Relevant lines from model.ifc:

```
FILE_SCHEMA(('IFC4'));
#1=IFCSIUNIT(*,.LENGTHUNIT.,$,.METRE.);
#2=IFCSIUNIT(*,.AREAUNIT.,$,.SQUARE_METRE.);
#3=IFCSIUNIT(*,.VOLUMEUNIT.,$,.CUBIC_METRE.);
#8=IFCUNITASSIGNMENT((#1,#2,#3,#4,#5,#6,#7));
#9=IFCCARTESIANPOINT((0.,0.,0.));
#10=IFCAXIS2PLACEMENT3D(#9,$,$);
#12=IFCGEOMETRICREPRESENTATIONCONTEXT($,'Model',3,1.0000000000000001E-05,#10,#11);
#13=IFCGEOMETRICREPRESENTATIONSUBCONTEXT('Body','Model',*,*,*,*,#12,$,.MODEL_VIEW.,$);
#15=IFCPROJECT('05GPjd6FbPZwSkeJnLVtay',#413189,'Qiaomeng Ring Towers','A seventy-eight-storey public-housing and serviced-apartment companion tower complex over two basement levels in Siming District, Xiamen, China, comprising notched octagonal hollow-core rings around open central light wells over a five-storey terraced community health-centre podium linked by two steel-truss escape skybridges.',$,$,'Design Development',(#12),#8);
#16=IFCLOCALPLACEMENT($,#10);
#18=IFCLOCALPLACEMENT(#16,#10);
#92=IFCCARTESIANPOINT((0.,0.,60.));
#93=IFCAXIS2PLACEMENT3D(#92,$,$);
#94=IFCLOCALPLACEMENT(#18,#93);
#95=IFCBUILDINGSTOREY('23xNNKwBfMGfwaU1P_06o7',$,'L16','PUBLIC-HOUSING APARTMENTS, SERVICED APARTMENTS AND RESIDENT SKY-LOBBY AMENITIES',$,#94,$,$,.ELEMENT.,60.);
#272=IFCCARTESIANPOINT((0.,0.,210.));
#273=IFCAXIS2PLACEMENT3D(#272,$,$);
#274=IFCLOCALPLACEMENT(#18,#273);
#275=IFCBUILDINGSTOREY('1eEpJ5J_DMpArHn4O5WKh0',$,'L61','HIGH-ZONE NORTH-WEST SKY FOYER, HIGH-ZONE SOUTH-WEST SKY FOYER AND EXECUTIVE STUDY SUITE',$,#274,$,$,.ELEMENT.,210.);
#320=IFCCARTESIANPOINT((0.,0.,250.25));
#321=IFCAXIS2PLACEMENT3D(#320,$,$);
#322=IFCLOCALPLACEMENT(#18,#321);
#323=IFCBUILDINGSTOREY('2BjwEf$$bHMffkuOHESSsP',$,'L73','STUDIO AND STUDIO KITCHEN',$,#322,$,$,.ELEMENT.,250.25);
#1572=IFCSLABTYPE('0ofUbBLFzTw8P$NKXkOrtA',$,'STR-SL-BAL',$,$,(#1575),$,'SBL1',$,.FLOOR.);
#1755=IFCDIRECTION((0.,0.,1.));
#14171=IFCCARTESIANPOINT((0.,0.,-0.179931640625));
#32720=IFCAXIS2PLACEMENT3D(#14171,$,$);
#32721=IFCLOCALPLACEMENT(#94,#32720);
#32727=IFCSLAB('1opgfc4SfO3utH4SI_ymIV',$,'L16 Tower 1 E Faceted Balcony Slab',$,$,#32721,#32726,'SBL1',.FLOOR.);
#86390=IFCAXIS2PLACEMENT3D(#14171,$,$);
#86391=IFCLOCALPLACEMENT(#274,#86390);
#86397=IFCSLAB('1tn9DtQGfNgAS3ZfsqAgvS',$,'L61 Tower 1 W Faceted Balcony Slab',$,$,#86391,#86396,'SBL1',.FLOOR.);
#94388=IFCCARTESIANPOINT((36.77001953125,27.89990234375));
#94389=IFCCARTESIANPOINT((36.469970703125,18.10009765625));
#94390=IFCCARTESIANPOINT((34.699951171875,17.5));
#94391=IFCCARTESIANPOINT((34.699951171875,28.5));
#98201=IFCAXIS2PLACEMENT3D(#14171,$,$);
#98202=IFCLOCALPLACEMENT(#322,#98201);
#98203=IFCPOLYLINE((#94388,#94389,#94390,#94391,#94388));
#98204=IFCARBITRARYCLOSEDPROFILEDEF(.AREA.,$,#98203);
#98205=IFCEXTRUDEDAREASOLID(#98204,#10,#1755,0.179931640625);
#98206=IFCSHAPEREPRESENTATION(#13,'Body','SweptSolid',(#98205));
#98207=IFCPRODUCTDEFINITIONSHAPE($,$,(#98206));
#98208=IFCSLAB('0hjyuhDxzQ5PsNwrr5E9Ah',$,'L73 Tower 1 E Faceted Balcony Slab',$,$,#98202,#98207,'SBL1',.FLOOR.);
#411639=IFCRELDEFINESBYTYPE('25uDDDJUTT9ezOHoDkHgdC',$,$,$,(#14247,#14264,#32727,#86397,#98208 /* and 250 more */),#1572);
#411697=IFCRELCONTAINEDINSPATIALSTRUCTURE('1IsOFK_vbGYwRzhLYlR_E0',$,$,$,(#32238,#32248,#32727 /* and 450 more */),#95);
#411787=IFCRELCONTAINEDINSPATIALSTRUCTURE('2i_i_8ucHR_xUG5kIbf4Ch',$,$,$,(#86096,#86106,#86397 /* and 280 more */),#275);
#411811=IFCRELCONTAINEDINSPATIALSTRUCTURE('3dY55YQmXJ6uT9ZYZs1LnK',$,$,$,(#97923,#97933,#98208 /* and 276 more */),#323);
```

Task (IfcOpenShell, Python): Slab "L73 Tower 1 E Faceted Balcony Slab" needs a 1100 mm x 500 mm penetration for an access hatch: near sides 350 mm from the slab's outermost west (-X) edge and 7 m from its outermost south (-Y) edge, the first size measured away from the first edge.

```python
import numpy as np
import ifcopenshell
import ifcopenshell.api.feature
import ifcopenshell.api.geometry
import ifcopenshell.api.root
import ifcopenshell.geom
import ifcopenshell.util.placement
import ifcopenshell.util.representation
import ifcopenshell.util.shape
import ifcopenshell.util.unit

model = ifcopenshell.open("model.ifc")
unit_scale = ifcopenshell.util.unit.calculate_unit_scale(model)
settings = ifcopenshell.geom.settings()


def volume(element):
    """Net volume in cubic metres, openings subtracted."""
    shape = ifcopenshell.geom.create_shape(settings, element)
    return ifcopenshell.util.shape.get_volume(shape.geometry)


slab = model.by_guid("0hjyuhDxzQ5PsNwrr5E9Ah")
before = volume(slab)

# Extent in the slab's own axes, in metres. The edges named are its -X and -Y sides.
slab_shape = ifcopenshell.geom.create_shape(settings, slab)
vertices = ifcopenshell.util.shape.get_vertices(slab_shape.geometry)
x_min, y_min, bottom = vertices.min(axis=0)
top = vertices[:, 2].max()

opening = ifcopenshell.api.root.create_entity(model, ifc_class="IfcOpeningElement", name="Access hatch opening", predefined_type="OPENING")
context = ifcopenshell.util.representation.get_context(model, "Model", "Body", "MODEL_VIEW")
width, depth = 1.1, 0.5
outline = [(0.0, 0.0), (width, 0.0), (width, depth), (0.0, depth), (0.0, 0.0)]
# Overshoot both faces by 50 mm so the cut is clean.
shape = ifcopenshell.api.geometry.add_slab_representation(
    model, context=context, depth=top - bottom + 0.1, polyline=outline
)
ifcopenshell.api.geometry.assign_representation(model, product=opening, representation=shape)

matrix = ifcopenshell.util.placement.get_local_placement(slab.ObjectPlacement)
matrix[:, 3] = matrix @ np.append(np.array([x_min + 0.35, y_min + 7, bottom - 0.05]) / unit_scale, 1.0)
ifcopenshell.api.geometry.edit_object_placement(model, product=opening, matrix=matrix, is_si=False)
ifcopenshell.api.feature.add_feature(model, feature=opening, element=slab)

after = volume(slab)

print(f"slab volume {before:.3f} -> {after:.3f} m3")

model.write("model_v2.ifc")
```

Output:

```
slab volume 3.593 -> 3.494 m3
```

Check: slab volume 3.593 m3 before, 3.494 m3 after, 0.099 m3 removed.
